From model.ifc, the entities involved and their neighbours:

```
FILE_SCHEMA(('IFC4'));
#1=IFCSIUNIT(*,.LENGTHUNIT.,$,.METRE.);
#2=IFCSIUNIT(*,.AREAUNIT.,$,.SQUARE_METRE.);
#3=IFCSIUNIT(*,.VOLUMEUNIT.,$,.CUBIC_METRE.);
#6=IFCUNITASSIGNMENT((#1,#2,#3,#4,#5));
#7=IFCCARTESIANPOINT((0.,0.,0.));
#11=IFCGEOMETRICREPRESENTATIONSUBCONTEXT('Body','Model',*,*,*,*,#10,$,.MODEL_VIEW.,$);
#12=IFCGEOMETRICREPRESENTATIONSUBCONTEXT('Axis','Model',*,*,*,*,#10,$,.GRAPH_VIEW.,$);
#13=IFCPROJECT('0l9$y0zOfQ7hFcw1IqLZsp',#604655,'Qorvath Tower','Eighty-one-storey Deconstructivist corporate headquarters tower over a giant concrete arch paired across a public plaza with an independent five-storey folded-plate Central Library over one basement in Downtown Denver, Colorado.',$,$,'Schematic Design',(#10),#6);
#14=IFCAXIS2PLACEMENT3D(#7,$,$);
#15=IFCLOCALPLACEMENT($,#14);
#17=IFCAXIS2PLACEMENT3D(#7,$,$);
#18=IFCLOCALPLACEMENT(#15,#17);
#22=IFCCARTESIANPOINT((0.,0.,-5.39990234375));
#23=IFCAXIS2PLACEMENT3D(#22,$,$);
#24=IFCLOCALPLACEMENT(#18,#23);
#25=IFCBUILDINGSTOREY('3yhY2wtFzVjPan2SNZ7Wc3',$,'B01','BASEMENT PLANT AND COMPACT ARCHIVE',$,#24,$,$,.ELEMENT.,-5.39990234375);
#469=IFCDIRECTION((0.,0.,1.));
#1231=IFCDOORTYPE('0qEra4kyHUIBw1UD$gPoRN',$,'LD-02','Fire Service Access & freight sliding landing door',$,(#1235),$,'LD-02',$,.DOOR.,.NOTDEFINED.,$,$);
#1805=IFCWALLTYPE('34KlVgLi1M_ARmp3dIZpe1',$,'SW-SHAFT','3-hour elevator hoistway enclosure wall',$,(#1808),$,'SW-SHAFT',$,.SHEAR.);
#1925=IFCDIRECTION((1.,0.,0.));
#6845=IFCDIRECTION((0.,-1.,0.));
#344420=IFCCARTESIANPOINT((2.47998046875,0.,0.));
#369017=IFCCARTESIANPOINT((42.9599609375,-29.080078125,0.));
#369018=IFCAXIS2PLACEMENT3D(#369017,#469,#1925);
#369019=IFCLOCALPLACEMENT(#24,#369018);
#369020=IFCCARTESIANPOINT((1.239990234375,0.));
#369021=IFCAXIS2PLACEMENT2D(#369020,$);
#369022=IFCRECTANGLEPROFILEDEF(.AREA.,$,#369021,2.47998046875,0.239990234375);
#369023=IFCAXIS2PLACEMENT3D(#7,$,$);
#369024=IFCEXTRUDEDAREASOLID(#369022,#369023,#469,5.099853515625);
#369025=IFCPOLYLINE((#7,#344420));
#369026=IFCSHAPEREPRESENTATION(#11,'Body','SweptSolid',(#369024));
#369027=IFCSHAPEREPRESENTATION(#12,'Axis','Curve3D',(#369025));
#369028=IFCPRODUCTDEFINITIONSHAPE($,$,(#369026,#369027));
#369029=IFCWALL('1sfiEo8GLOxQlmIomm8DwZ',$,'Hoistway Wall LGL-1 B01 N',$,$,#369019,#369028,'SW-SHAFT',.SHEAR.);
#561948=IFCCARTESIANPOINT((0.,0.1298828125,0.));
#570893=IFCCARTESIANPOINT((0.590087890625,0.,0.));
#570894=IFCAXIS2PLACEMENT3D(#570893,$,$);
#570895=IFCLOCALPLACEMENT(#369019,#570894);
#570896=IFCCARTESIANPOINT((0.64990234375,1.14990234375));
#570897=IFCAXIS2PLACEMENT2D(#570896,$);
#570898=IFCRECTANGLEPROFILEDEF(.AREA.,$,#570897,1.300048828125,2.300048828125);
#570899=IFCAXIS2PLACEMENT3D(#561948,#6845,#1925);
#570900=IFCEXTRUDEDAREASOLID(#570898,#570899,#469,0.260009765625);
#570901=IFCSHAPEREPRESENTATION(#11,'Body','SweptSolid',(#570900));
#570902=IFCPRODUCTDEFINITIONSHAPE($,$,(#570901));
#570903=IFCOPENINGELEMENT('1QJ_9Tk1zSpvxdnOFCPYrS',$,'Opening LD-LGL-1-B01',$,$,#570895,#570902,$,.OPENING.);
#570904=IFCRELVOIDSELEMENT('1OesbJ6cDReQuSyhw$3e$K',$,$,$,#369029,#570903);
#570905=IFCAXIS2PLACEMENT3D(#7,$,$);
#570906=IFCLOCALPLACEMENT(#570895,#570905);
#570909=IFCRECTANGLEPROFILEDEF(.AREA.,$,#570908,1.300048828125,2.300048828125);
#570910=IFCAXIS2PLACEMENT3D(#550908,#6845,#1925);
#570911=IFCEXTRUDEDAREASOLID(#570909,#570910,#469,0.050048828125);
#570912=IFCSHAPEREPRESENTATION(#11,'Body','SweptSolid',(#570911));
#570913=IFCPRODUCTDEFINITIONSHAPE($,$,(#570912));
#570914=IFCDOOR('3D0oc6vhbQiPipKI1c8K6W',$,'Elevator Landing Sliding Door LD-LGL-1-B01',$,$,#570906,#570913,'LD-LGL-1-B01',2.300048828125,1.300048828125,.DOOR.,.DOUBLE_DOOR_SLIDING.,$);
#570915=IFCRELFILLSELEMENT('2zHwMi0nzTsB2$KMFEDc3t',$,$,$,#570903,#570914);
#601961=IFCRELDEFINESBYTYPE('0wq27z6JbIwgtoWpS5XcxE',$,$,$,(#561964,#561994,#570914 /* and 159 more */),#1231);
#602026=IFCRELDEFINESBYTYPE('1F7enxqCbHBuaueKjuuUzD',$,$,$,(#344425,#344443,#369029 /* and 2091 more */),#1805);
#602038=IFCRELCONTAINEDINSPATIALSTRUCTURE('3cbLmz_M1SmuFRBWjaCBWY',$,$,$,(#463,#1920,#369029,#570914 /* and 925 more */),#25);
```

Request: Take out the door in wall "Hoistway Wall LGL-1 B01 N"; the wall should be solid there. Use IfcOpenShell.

```python
import ifcopenshell
import ifcopenshell.api.feature
import ifcopenshell.api.root
import ifcopenshell.geom
import ifcopenshell.util.shape

model = ifcopenshell.open("model.ifc")
settings = ifcopenshell.geom.settings()


def volume(element):
    """Net volume in cubic metres, openings subtracted."""
    shape = ifcopenshell.geom.create_shape(settings, element)
    return ifcopenshell.util.shape.get_volume(shape.geometry)


door = model.by_guid("3D0oc6vhbQiPipKI1c8K6W")
opening = door.FillsVoids[0].RelatingOpeningElement
wall = opening.VoidsElements[0].RelatingBuildingElement
before = volume(wall)

ifcopenshell.api.root.remove_product(model, product=door)
ifcopenshell.api.feature.remove_feature(model, feature=opening)

after = volume(wall)

print(f"wall volume {before:.3f} -> {after:.3f} m3")

model.write("model_updated.ifc")
```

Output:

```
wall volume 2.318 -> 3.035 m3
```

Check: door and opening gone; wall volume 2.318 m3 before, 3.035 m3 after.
